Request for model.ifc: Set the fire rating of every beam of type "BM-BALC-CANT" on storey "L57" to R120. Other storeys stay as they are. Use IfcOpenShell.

First a look at what the model holds.

```python
import ifcopenshell
import ifcopenshell.util.element

model = ifcopenshell.open("model.ifc")
print(model.schema)
storey = next(s for s in model.by_type("IfcBuildingStorey") if s.Name == "L57")
beams = [e for e in ifcopenshell.util.element.get_decomposition(storey) if e.is_a("IfcBeam")]
seen = {}
for e in beams:
    element_type = ifcopenshell.util.element.get_type(e)
    key = (element_type.Name if element_type != e and element_type else None, ifcopenshell.util.element.get_pset(e, "Pset_BeamCommon", "FireRating"))
    seen[key] = seen.get(key, 0) + 1
for (name, value), count in sorted(seen.items(), key=str):
    print(count, "x", name, "|", value)
```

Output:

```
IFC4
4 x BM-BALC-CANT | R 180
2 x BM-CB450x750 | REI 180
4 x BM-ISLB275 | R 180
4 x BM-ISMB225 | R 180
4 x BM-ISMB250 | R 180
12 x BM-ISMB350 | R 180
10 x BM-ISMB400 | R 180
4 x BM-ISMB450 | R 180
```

```python
import ifcopenshell
import ifcopenshell.api.pset
import ifcopenshell.util.element

model = ifcopenshell.open("model.ifc")

storey = next(s for s in model.by_type("IfcBuildingStorey") if s.Name == "L57")
beams = [e for e in ifcopenshell.util.element.get_decomposition(storey) if e.is_a("IfcBeam")]

count = 0
for e in beams:
    element_type = ifcopenshell.util.element.get_type(e)
    if element_type in (None, e) or element_type.Name != "BM-BALC-CANT":
        continue
    found = ifcopenshell.util.element.get_pset(e, "Pset_BeamCommon", should_inherit=False)
    if found:
        pset = model.by_id(found["id"])
        if len(ifcopenshell.util.element.get_elements_by_pset(pset)) > 1:
            pset = ifcopenshell.api.pset.unshare_pset(model, products=[e], pset=pset)[0]
    else:
        pset = ifcopenshell.api.pset.add_pset(model, product=e, name="Pset_BeamCommon")
    ifcopenshell.api.pset.edit_pset(model, pset=pset, properties={"FireRating": "R120"})
    count += 1

print(count, "beams updated")

model.write("model_edited.ifc")
```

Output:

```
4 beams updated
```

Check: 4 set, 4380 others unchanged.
